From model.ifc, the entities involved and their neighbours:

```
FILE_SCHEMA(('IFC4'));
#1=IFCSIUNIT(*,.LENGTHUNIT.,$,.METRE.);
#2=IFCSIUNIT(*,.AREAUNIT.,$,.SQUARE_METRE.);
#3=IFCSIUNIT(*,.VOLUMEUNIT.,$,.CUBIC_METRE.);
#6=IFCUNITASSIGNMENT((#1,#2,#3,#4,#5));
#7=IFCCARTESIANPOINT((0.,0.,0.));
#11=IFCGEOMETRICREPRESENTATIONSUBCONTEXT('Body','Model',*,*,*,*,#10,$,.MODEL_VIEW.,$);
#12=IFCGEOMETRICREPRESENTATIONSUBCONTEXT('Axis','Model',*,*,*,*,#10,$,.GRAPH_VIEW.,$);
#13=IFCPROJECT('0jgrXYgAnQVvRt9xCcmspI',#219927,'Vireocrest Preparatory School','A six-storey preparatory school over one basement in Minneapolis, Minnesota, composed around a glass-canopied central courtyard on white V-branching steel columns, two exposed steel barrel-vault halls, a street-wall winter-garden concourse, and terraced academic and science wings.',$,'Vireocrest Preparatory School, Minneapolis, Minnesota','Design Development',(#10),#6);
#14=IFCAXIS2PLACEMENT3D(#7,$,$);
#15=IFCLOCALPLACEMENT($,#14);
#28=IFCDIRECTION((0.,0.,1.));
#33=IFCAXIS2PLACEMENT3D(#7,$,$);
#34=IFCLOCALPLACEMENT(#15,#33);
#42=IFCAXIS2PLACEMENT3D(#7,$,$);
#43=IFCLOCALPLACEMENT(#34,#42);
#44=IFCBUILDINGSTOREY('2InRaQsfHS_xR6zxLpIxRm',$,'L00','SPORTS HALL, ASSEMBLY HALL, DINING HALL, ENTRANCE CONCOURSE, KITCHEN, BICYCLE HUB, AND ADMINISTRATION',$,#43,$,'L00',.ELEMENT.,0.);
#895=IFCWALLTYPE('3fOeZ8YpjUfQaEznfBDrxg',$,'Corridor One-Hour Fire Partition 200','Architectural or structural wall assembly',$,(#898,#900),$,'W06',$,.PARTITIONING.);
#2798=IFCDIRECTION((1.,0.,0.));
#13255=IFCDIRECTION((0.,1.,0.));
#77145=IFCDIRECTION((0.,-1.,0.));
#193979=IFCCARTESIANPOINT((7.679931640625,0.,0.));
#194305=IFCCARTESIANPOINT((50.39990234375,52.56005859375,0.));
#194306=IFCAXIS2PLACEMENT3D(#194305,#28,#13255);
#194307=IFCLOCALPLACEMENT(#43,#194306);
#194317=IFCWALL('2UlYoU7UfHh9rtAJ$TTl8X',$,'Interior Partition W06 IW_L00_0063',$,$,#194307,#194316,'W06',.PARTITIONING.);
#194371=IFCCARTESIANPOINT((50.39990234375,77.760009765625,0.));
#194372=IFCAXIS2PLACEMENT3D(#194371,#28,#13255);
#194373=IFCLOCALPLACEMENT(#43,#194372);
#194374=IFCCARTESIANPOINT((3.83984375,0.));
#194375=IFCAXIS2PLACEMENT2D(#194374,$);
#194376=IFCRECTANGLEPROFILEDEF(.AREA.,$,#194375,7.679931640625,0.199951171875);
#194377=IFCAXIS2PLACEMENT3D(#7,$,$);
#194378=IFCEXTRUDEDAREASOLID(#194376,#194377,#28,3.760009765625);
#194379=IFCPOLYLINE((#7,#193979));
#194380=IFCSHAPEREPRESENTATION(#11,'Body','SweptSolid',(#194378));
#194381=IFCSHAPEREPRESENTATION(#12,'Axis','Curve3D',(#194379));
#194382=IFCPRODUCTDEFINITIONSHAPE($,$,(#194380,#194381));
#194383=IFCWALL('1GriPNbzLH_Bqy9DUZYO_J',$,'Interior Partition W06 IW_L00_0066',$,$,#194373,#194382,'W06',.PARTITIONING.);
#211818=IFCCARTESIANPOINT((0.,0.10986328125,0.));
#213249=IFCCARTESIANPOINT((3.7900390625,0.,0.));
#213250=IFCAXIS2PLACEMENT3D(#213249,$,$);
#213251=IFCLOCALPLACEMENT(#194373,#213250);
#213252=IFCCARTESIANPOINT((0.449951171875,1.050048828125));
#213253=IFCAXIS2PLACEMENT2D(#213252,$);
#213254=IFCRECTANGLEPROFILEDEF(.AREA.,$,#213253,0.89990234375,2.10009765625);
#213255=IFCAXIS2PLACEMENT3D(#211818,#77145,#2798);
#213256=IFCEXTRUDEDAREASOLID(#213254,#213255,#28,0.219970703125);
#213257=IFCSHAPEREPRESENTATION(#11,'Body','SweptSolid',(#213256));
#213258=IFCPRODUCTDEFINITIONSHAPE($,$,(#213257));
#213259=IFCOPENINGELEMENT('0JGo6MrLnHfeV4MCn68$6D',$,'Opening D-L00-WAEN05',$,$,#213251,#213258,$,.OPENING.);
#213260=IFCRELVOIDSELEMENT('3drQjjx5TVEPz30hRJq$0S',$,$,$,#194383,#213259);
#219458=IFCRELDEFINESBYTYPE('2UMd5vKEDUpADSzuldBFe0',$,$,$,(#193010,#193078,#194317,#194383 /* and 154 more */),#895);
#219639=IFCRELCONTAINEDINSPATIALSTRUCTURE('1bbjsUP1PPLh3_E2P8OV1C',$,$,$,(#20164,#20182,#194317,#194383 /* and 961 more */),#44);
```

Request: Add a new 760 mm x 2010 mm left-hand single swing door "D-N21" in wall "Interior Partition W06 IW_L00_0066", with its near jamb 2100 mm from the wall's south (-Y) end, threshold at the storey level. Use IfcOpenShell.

```python
import numpy as np
import ifcopenshell
import ifcopenshell.api.feature
import ifcopenshell.api.geometry
import ifcopenshell.api.root
import ifcopenshell.api.spatial
import ifcopenshell.geom
import ifcopenshell.util.element
import ifcopenshell.util.placement
import ifcopenshell.util.representation
import ifcopenshell.util.shape
import ifcopenshell.util.unit

model = ifcopenshell.open("model.ifc")
unit_scale = ifcopenshell.util.unit.calculate_unit_scale(model)
settings = ifcopenshell.geom.settings()


def volume(element):
    """Net volume in cubic metres, openings subtracted."""
    shape = ifcopenshell.geom.create_shape(settings, element)
    return ifcopenshell.util.shape.get_volume(shape.geometry)


wall = model.by_guid("1GriPNbzLH_Bqy9DUZYO_J")
storey = ifcopenshell.util.element.get_container(wall, ifc_class="IfcBuildingStorey")
context = ifcopenshell.util.representation.get_context(model, "Model", "Body", "MODEL_VIEW")
before = volume(wall)

width, height, from_end, sill = 0.76, 2.01, 2.1, 0.0  # metres

# The wall runs along its own X axis, and the end named is its -X end.
wall_shape = ifcopenshell.geom.create_shape(settings, wall)
x, y, z = ifcopenshell.util.shape.get_vertices(wall_shape.geometry).T
start = x.min() + from_end
face, thickness = float(y.min()), float(y.max() - y.min())
wall_matrix = ifcopenshell.util.placement.get_local_placement(wall.ObjectPlacement)
level = ifcopenshell.util.placement.get_local_placement(storey.ObjectPlacement)[2, 3]


def in_wall(x, y):
    """Placement at x, y metres in the wall's axes, at sill height."""
    matrix = wall_matrix.copy()
    matrix[:, 3] = wall_matrix @ np.array([x / unit_scale, y / unit_scale, 0.0, 1.0])
    matrix[2, 3] = level + sill / unit_scale
    return matrix


# Opening: a box that overshoots both wall faces by 50 mm.
opening = ifcopenshell.api.root.create_entity(model, ifc_class="IfcOpeningElement", predefined_type="OPENING")
box = ifcopenshell.api.geometry.add_wall_representation(
    model, context=context, length=width, height=height, thickness=thickness + 0.1
)
ifcopenshell.api.geometry.assign_representation(model, product=opening, representation=box)
ifcopenshell.api.geometry.edit_object_placement(model, product=opening, matrix=in_wall(start, face - 0.05), is_si=False)
ifcopenshell.api.feature.add_feature(model, feature=opening, element=wall)

door = ifcopenshell.api.root.create_entity(model, ifc_class="IfcDoor", name="D-N21", predefined_type="DOOR")
door.OverallWidth, door.OverallHeight = width / unit_scale, height / unit_scale
door.OperationType = "SINGLE_SWING_LEFT"
body = ifcopenshell.api.geometry.add_door_representation(
    model,
    context=context,
    overall_width=door.OverallWidth,
    overall_height=door.OverallHeight,
    operation_type="SINGLE_SWING_LEFT",
    lining_properties={"LiningDepth": thickness / unit_scale, "ThresholdDepth": thickness / unit_scale},
)
ifcopenshell.api.geometry.assign_representation(model, product=door, representation=body)
ifcopenshell.api.spatial.assign_container(model, products=[door], relating_structure=storey)
ifcopenshell.api.feature.add_filling(model, opening=opening, element=door)

# The lining spans the wall, so the door starts at the wall face.
ifcopenshell.api.geometry.edit_object_placement(model, product=door, matrix=in_wall(start, face), is_si=False)

after = volume(wall)

print(f"wall volume {before:.3f} -> {after:.3f} m3")

model.write("model_v2.ifc")
```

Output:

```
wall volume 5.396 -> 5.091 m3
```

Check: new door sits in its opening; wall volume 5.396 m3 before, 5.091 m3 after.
